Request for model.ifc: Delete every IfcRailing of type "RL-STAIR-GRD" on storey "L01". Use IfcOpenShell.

First a look at what the model holds.

```python
import ifcopenshell
import ifcopenshell.util.element

model = ifcopenshell.open("model.ifc")
print(model.schema)
storey = next(s for s in model.by_type("IfcBuildingStorey") if s.Name == "L01")
railings = [e for e in ifcopenshell.util.element.get_decomposition(storey) if e.is_a("IfcRailing")]
seen = {}
for e in railings:
    element_type = ifcopenshell.util.element.get_type(e)
    name = element_type.Name if element_type not in (None, e) else None
    seen[name] = seen.get(name, 0) + 1
for name, count in sorted(seen.items(), key=str):
    print(count, "x", name)
```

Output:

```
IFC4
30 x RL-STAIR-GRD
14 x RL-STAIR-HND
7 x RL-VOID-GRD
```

```python
import ifcopenshell
import ifcopenshell.api.root
import ifcopenshell.util.element

model = ifcopenshell.open("model.ifc")

storey = next(s for s in model.by_type("IfcBuildingStorey") if s.Name == "L01")
railings = [e for e in ifcopenshell.util.element.get_decomposition(storey) if e.is_a("IfcRailing")]
targets = [e for e in railings if (t := ifcopenshell.util.element.get_type(e)) not in (None, e) and t.Name == "RL-STAIR-GRD"]

for e in targets:
    ifcopenshell.api.root.remove_product(model, product=e)
print(len(targets), "removed")

model.write("model_v2.ifc")
```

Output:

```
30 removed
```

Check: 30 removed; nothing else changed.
